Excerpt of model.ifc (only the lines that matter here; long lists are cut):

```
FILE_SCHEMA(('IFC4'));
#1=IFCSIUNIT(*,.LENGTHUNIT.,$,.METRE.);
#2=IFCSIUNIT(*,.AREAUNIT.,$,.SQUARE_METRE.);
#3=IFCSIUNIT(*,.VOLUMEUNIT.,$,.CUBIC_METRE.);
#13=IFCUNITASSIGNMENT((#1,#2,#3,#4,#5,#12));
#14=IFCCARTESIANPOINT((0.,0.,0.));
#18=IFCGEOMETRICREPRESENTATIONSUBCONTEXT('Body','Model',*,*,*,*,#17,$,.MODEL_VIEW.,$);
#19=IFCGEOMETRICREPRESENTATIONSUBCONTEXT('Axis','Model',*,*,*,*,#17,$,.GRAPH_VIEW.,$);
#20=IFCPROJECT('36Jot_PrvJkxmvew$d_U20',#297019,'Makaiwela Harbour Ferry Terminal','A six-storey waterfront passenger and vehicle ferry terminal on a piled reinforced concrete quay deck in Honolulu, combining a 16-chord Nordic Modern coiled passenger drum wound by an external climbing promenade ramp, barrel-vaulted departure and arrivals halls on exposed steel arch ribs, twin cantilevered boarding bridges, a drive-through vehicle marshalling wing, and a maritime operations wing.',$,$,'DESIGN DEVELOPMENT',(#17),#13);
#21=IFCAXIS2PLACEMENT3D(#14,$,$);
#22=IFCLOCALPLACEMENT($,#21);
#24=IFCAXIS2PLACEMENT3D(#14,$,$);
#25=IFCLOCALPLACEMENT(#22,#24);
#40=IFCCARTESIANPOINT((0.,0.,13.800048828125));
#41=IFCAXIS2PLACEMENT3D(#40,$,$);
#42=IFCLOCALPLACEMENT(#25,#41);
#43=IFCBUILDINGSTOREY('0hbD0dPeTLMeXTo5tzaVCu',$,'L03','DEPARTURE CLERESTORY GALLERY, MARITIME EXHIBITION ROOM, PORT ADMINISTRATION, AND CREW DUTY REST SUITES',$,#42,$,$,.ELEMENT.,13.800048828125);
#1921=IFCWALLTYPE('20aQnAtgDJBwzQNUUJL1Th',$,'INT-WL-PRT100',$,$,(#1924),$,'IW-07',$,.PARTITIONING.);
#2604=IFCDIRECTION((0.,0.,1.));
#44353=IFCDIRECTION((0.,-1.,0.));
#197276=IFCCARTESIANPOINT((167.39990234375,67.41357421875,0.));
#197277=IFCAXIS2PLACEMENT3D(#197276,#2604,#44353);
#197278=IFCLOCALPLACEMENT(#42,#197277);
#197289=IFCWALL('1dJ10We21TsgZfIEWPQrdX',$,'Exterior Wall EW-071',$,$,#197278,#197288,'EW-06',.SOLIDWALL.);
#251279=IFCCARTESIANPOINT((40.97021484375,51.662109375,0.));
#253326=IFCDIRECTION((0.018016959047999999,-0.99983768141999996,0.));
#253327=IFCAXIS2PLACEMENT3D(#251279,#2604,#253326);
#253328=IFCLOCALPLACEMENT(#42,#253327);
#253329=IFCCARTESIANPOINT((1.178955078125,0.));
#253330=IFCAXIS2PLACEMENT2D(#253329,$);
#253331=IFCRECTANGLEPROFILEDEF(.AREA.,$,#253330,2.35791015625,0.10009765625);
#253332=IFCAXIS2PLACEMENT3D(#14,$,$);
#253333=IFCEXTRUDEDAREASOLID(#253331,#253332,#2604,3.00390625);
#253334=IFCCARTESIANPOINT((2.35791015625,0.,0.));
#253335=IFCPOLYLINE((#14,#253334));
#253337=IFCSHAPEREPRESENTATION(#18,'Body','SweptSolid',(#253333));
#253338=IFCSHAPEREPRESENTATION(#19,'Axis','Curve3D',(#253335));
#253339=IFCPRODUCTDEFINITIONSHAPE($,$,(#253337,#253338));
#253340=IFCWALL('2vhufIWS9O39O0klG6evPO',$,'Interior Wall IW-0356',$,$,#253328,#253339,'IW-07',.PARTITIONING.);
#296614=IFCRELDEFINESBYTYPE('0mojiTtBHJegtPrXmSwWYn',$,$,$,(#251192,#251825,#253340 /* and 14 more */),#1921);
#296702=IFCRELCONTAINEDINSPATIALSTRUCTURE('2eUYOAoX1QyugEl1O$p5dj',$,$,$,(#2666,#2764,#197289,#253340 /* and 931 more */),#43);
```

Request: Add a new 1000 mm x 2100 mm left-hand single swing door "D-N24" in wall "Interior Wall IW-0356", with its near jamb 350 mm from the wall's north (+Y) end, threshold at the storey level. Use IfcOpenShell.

```python
import numpy as np
import ifcopenshell
import ifcopenshell.api.feature
import ifcopenshell.api.geometry
import ifcopenshell.api.root
import ifcopenshell.api.spatial
import ifcopenshell.geom
import ifcopenshell.util.element
import ifcopenshell.util.placement
import ifcopenshell.util.representation
import ifcopenshell.util.shape
import ifcopenshell.util.unit

model = ifcopenshell.open("model.ifc")
unit_scale = ifcopenshell.util.unit.calculate_unit_scale(model)
settings = ifcopenshell.geom.settings()


def volume(element):
    """Net volume in cubic metres, openings subtracted."""
    shape = ifcopenshell.geom.create_shape(settings, element)
    return ifcopenshell.util.shape.get_volume(shape.geometry)


wall = model.by_guid("2vhufIWS9O39O0klG6evPO")
storey = ifcopenshell.util.element.get_container(wall, ifc_class="IfcBuildingStorey")
context = ifcopenshell.util.representation.get_context(model, "Model", "Body", "MODEL_VIEW")
before = volume(wall)

width, height, from_end, sill = 1, 2.1, 0.35, 0.0  # metres

# The wall runs along its own X axis, and the end named is its -X end.
wall_shape = ifcopenshell.geom.create_shape(settings, wall)
x, y, z = ifcopenshell.util.shape.get_vertices(wall_shape.geometry).T
start = x.min() + from_end
face, thickness = float(y.min()), float(y.max() - y.min())
wall_matrix = ifcopenshell.util.placement.get_local_placement(wall.ObjectPlacement)
level = ifcopenshell.util.placement.get_local_placement(storey.ObjectPlacement)[2, 3]


def in_wall(x, y):
    """Placement at x, y metres in the wall's axes, at sill height."""
    matrix = wall_matrix.copy()
    matrix[:, 3] = wall_matrix @ np.array([x / unit_scale, y / unit_scale, 0.0, 1.0])
    matrix[2, 3] = level + sill / unit_scale
    return matrix


# Opening: a box that overshoots both wall faces by 50 mm.
opening = ifcopenshell.api.root.create_entity(model, ifc_class="IfcOpeningElement", predefined_type="OPENING")
box = ifcopenshell.api.geometry.add_wall_representation(
    model, context=context, length=width, height=height, thickness=thickness + 0.1
)
ifcopenshell.api.geometry.assign_representation(model, product=opening, representation=box)
ifcopenshell.api.geometry.edit_object_placement(model, product=opening, matrix=in_wall(start, face - 0.05), is_si=False)
ifcopenshell.api.feature.add_feature(model, feature=opening, element=wall)

door = ifcopenshell.api.root.create_entity(model, ifc_class="IfcDoor", name="D-N24", predefined_type="DOOR")
door.OverallWidth, door.OverallHeight = width / unit_scale, height / unit_scale
door.OperationType = "SINGLE_SWING_LEFT"
body = ifcopenshell.api.geometry.add_door_representation(
    model,
    context=context,
    overall_width=door.OverallWidth,
    overall_height=door.OverallHeight,
    operation_type="SINGLE_SWING_LEFT",
    lining_properties={"LiningDepth": thickness / unit_scale, "ThresholdDepth": thickness / unit_scale},
)
ifcopenshell.api.geometry.assign_representation(model, product=door, representation=body)
ifcopenshell.api.spatial.assign_container(model, products=[door], relating_structure=storey)
ifcopenshell.api.feature.add_filling(model, opening=opening, element=door)

# The lining spans the wall, so the door starts at the wall face.
ifcopenshell.api.geometry.edit_object_placement(model, product=door, matrix=in_wall(start, face), is_si=False)

after = volume(wall)

print(f"wall volume {before:.3f} -> {after:.3f} m3")

model.write("model_updated.ifc")
```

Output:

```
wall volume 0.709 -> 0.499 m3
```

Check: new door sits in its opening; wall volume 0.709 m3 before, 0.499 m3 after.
